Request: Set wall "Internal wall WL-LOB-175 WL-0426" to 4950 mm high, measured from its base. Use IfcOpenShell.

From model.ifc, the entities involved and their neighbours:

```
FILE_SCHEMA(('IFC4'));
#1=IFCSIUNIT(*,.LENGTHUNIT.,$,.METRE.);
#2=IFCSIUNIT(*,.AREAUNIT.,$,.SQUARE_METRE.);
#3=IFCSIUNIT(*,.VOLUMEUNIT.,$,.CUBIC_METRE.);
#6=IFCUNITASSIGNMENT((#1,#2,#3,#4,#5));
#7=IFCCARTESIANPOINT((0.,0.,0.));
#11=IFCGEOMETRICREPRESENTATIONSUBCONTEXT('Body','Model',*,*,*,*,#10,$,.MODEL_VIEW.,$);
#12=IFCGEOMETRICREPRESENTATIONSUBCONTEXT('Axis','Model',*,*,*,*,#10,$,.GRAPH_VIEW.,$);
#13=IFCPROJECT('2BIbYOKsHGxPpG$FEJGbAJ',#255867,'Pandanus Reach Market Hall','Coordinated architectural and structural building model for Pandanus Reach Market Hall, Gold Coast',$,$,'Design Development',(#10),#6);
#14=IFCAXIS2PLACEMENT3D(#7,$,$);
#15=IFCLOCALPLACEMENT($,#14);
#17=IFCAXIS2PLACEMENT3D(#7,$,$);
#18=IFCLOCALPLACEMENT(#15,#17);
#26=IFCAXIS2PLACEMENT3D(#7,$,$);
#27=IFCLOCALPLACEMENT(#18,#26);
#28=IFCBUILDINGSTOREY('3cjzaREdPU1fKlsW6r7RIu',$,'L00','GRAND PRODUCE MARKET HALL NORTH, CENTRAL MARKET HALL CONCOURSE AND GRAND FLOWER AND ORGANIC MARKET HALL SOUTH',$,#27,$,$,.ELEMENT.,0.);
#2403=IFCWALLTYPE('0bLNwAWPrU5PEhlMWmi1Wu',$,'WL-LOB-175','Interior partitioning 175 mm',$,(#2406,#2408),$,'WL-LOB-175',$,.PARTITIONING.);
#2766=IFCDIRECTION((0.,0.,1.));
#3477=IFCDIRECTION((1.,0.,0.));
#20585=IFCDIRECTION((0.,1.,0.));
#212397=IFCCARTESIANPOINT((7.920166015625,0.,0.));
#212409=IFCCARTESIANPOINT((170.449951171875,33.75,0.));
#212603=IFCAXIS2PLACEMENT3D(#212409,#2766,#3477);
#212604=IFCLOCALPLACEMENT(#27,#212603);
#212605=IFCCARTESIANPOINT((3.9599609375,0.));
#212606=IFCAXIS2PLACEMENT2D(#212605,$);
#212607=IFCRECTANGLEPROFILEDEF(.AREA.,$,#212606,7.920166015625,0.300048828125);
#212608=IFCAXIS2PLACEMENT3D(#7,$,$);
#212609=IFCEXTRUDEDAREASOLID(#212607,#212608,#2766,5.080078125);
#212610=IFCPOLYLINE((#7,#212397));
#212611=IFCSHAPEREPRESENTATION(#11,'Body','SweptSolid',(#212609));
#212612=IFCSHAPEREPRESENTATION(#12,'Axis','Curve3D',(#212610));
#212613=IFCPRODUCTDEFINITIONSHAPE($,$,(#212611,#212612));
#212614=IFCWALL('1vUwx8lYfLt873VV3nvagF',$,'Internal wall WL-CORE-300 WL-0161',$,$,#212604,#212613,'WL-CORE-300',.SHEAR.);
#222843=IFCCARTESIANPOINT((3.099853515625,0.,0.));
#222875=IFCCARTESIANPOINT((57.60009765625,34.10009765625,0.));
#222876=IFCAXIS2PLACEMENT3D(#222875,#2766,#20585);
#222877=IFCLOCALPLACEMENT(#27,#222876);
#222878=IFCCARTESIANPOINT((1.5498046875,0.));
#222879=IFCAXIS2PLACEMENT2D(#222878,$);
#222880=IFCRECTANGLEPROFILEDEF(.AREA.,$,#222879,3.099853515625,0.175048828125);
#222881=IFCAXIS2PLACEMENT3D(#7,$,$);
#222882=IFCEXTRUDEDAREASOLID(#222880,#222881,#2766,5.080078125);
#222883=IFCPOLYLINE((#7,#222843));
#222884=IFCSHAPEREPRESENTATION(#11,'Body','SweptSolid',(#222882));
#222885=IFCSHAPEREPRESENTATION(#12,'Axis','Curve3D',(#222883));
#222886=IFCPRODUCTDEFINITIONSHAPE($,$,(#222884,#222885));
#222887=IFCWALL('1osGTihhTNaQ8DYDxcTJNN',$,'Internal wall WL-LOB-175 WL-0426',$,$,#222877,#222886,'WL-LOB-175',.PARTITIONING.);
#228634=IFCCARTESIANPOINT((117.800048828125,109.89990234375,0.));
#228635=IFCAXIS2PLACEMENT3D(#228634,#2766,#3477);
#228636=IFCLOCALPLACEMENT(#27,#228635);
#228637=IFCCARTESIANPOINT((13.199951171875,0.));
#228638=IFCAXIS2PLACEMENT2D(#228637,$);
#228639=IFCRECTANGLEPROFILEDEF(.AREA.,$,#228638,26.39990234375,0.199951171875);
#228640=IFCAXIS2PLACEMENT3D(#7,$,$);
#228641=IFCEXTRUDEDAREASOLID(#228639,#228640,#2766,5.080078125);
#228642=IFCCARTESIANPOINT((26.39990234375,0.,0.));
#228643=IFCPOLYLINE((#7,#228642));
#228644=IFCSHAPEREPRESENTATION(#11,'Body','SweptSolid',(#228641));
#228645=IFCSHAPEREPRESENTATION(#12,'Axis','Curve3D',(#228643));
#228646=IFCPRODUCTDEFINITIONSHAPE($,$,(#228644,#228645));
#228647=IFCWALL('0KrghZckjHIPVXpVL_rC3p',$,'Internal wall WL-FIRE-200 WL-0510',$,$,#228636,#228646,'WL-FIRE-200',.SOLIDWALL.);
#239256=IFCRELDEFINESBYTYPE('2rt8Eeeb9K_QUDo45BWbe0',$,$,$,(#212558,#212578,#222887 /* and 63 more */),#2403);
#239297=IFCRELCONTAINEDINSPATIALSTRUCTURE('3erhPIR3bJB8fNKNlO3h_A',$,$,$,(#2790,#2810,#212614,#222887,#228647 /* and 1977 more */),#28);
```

```python
import ifcopenshell
import ifcopenshell.geom
import ifcopenshell.util.representation
import ifcopenshell.util.shape
import ifcopenshell.util.unit

model = ifcopenshell.open("model.ifc")
unit_scale = ifcopenshell.util.unit.calculate_unit_scale(model)
settings = ifcopenshell.geom.settings()


def volume(element):
    """Net volume in cubic metres, openings subtracted."""
    shape = ifcopenshell.geom.create_shape(settings, element)
    return ifcopenshell.util.shape.get_volume(shape.geometry)


wall = model.by_id(222887)
before = volume(wall)

body = ifcopenshell.util.representation.get_representation(wall, "Model", "Body")
solid = body.Items[0]
old_height = solid.Depth
solid.Depth = 4.95 / unit_scale
after = volume(wall)

print(f"height {old_height:g} -> {solid.Depth:g}, volume {before:.3f} -> {after:.3f} m3")

model.write("model_v2.ifc")
```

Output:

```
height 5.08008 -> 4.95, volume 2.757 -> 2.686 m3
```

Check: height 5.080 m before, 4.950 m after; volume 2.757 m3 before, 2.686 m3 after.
